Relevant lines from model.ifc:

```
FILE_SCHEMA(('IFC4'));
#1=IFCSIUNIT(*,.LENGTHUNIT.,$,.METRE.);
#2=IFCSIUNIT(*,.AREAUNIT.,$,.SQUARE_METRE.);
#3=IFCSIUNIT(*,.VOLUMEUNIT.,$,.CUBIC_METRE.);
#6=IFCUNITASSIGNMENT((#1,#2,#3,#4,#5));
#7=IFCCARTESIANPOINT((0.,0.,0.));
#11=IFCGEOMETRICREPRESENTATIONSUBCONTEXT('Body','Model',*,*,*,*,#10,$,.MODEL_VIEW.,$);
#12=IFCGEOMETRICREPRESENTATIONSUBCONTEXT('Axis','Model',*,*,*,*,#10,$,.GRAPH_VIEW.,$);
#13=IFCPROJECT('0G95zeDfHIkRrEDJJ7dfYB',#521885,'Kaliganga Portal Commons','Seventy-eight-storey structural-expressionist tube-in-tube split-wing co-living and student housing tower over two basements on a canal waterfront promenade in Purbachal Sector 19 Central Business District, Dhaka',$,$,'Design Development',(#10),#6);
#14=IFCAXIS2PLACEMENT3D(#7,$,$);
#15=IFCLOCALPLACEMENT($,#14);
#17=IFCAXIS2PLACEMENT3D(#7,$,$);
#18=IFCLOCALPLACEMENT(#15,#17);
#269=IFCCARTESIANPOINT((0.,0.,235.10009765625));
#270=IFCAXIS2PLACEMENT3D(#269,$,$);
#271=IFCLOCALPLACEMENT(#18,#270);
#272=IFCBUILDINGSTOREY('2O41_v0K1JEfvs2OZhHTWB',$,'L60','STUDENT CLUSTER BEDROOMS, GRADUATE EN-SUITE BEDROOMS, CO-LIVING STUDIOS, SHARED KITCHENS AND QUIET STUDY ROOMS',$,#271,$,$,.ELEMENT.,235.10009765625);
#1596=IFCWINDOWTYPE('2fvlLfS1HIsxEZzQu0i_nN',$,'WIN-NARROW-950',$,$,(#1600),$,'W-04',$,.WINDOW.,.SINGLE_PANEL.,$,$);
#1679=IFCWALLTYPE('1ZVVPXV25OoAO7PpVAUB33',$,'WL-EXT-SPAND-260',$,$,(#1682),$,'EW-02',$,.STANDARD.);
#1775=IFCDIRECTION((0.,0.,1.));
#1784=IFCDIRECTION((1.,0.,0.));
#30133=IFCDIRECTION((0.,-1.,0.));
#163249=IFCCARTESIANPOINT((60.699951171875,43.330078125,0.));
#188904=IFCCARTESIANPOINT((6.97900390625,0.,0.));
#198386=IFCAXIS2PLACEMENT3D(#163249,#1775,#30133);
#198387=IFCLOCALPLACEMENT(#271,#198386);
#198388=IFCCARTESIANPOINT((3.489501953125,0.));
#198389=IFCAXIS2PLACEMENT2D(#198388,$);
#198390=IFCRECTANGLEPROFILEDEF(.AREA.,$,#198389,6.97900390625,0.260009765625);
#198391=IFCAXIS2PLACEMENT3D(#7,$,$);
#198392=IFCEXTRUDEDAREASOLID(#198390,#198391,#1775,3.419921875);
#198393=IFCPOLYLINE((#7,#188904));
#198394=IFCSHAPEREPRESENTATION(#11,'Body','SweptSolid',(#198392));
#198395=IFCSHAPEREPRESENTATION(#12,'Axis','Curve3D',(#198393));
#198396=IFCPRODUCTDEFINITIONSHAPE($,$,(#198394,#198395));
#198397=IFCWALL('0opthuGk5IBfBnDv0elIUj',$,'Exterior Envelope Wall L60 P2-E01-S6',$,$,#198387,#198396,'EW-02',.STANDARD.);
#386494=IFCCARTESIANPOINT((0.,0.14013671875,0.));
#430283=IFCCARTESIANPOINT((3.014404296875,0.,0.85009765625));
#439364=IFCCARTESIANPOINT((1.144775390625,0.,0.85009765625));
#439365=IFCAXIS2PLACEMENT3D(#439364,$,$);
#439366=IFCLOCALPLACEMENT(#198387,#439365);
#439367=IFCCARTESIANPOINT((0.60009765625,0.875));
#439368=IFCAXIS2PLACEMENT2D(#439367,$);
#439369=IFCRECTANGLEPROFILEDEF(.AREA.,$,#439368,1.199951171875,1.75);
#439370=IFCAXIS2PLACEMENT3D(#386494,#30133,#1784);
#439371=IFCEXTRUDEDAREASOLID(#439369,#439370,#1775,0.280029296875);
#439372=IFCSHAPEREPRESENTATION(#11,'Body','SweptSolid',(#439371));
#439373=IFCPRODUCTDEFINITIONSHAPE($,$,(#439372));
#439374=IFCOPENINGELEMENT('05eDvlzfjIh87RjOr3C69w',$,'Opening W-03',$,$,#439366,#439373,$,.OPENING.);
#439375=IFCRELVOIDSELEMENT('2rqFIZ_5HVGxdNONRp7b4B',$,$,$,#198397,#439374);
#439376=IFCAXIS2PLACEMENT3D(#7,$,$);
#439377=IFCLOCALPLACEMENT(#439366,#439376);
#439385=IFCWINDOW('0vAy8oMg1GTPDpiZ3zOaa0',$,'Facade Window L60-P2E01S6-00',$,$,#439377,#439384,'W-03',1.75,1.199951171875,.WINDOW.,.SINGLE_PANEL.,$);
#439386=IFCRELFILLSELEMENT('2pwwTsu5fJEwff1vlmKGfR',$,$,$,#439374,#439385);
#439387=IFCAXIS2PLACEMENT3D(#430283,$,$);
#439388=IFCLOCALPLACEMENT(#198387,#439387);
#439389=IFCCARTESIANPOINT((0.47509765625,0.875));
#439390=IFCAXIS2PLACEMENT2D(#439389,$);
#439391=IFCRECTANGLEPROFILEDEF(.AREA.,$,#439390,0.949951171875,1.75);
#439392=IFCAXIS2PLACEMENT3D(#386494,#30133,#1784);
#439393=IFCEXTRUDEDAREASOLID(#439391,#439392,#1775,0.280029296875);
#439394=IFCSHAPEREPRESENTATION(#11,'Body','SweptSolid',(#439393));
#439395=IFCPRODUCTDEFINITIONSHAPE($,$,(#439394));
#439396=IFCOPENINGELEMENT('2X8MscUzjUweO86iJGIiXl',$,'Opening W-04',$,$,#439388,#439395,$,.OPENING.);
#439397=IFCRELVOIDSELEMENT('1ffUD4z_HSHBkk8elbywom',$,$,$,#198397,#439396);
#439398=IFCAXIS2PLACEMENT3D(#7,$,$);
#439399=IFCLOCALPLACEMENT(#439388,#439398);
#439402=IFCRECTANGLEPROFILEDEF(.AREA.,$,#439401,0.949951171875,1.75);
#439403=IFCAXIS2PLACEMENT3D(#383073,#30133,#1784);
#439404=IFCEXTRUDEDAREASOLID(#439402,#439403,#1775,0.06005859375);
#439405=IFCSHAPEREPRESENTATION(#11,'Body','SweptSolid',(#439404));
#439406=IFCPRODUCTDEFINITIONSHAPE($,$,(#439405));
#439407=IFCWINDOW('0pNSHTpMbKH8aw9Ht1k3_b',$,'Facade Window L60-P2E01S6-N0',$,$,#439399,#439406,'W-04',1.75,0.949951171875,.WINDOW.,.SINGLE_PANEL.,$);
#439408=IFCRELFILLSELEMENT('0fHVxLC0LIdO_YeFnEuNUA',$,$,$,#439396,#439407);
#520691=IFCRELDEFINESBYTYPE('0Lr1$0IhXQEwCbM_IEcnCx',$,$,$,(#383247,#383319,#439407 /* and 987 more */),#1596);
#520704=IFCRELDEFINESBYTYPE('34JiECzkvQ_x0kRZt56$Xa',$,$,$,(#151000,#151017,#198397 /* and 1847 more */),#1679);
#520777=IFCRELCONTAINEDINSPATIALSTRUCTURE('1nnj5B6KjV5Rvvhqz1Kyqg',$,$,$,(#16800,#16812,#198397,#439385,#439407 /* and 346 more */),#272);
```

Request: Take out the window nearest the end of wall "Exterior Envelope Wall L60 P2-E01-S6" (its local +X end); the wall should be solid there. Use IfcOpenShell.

```python
import ifcopenshell
import ifcopenshell.api.feature
import ifcopenshell.api.root
import ifcopenshell.geom
import ifcopenshell.util.shape

model = ifcopenshell.open("model.ifc")
settings = ifcopenshell.geom.settings()


def volume(element):
    """Net volume in cubic metres, openings subtracted."""
    shape = ifcopenshell.geom.create_shape(settings, element)
    return ifcopenshell.util.shape.get_volume(shape.geometry)


window = model.by_guid("0pNSHTpMbKH8aw9Ht1k3_b")
opening = window.FillsVoids[0].RelatingOpeningElement
wall = opening.VoidsElements[0].RelatingBuildingElement
before = volume(wall)

ifcopenshell.api.root.remove_product(model, product=window)
ifcopenshell.api.feature.remove_feature(model, feature=opening)

after = volume(wall)

print(f"wall volume {before:.3f} -> {after:.3f} m3")

model.write("model_edited.ifc")
```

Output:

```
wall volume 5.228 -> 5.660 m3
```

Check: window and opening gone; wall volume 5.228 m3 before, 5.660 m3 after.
